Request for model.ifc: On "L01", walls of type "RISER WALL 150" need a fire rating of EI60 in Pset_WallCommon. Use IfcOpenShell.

First a look at what the model holds.

```python
import ifcopenshell
import ifcopenshell.util.element

model = ifcopenshell.open("model.ifc")
print(model.schema)
storey = next(s for s in model.by_type("IfcBuildingStorey") if s.Name == "L01")
walls = [e for e in ifcopenshell.util.element.get_decomposition(storey) if e.is_a("IfcWall")]
seen = {}
for e in walls:
    element_type = ifcopenshell.util.element.get_type(e)
    key = (element_type.Name if element_type != e and element_type else None, ifcopenshell.util.element.get_pset(e, "Pset_WallCommon", "FireRating"))
    seen[key] = seen.get(key, 0) + 1
for (name, value), count in sorted(seen.items(), key=str):
    print(count, "x", name, "|", value)
```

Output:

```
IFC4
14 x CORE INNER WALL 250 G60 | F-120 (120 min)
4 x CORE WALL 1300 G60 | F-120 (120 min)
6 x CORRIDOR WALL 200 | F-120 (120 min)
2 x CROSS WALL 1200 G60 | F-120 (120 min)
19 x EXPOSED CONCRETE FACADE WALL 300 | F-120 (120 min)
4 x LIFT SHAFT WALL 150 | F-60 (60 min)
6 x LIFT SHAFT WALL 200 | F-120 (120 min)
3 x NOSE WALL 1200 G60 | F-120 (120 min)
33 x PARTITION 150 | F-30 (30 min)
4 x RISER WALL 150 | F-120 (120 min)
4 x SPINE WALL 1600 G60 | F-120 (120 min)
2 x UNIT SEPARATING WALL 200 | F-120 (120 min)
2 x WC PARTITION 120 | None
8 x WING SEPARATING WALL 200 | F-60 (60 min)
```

```python
import ifcopenshell
import ifcopenshell.api.pset
import ifcopenshell.util.element

model = ifcopenshell.open("model.ifc")

storey = next(s for s in model.by_type("IfcBuildingStorey") if s.Name == "L01")
walls = [e for e in ifcopenshell.util.element.get_decomposition(storey) if e.is_a("IfcWall")]

count = 0
for e in walls:
    element_type = ifcopenshell.util.element.get_type(e)
    if element_type in (None, e) or element_type.Name != "RISER WALL 150":
        continue
    found = ifcopenshell.util.element.get_pset(e, "Pset_WallCommon", should_inherit=False)
    if found:
        pset = model.by_id(found["id"])
        if len(ifcopenshell.util.element.get_elements_by_pset(pset)) > 1:
            pset = ifcopenshell.api.pset.unshare_pset(model, products=[e], pset=pset)[0]
    else:
        pset = ifcopenshell.api.pset.add_pset(model, product=e, name="Pset_WallCommon")
    ifcopenshell.api.pset.edit_pset(model, pset=pset, properties={"FireRating": "EI60"})
    count += 1

print(count, "walls updated")

model.write("model_updated.ifc")
```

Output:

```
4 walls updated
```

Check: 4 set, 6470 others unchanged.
